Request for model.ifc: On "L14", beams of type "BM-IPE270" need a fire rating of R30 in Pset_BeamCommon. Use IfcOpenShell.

First a look at what the model holds.

```python
import ifcopenshell
import ifcopenshell.util.element

model = ifcopenshell.open("model.ifc")
print(model.schema)
storey = next(s for s in model.by_type("IfcBuildingStorey") if s.Name == "L14")
beams = [e for e in ifcopenshell.util.element.get_decomposition(storey) if e.is_a("IfcBeam")]
seen = {}
for e in beams:
    element_type = ifcopenshell.util.element.get_type(e)
    key = (element_type.Name if element_type != e and element_type else None, ifcopenshell.util.element.get_pset(e, "Pset_BeamCommon", "FireRating"))
    seen[key] = seen.get(key, 0) + 1
for (name, value), count in sorted(seen.items(), key=str):
    print(count, "x", name, "|", value)
```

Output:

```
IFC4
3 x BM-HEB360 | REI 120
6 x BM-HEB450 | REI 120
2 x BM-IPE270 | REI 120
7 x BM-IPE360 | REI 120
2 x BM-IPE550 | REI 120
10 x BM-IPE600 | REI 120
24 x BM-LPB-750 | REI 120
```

```python
import ifcopenshell
import ifcopenshell.api.pset
import ifcopenshell.util.element

model = ifcopenshell.open("model.ifc")

storey = next(s for s in model.by_type("IfcBuildingStorey") if s.Name == "L14")
beams = [e for e in ifcopenshell.util.element.get_decomposition(storey) if e.is_a("IfcBeam")]

count = 0
for e in beams:
    element_type = ifcopenshell.util.element.get_type(e)
    if element_type in (None, e) or element_type.Name != "BM-IPE270":
        continue
    found = ifcopenshell.util.element.get_pset(e, "Pset_BeamCommon", should_inherit=False)
    if found:
        pset = model.by_id(found["id"])
        if len(ifcopenshell.util.element.get_elements_by_pset(pset)) > 1:
            pset = ifcopenshell.api.pset.unshare_pset(model, products=[e], pset=pset)[0]
    else:
        pset = ifcopenshell.api.pset.add_pset(model, product=e, name="Pset_BeamCommon")
    ifcopenshell.api.pset.edit_pset(model, pset=pset, properties={"FireRating": "R30"})
    count += 1

print(count, "beams updated")

model.write("model_v2.ifc")
```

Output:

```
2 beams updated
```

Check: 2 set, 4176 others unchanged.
